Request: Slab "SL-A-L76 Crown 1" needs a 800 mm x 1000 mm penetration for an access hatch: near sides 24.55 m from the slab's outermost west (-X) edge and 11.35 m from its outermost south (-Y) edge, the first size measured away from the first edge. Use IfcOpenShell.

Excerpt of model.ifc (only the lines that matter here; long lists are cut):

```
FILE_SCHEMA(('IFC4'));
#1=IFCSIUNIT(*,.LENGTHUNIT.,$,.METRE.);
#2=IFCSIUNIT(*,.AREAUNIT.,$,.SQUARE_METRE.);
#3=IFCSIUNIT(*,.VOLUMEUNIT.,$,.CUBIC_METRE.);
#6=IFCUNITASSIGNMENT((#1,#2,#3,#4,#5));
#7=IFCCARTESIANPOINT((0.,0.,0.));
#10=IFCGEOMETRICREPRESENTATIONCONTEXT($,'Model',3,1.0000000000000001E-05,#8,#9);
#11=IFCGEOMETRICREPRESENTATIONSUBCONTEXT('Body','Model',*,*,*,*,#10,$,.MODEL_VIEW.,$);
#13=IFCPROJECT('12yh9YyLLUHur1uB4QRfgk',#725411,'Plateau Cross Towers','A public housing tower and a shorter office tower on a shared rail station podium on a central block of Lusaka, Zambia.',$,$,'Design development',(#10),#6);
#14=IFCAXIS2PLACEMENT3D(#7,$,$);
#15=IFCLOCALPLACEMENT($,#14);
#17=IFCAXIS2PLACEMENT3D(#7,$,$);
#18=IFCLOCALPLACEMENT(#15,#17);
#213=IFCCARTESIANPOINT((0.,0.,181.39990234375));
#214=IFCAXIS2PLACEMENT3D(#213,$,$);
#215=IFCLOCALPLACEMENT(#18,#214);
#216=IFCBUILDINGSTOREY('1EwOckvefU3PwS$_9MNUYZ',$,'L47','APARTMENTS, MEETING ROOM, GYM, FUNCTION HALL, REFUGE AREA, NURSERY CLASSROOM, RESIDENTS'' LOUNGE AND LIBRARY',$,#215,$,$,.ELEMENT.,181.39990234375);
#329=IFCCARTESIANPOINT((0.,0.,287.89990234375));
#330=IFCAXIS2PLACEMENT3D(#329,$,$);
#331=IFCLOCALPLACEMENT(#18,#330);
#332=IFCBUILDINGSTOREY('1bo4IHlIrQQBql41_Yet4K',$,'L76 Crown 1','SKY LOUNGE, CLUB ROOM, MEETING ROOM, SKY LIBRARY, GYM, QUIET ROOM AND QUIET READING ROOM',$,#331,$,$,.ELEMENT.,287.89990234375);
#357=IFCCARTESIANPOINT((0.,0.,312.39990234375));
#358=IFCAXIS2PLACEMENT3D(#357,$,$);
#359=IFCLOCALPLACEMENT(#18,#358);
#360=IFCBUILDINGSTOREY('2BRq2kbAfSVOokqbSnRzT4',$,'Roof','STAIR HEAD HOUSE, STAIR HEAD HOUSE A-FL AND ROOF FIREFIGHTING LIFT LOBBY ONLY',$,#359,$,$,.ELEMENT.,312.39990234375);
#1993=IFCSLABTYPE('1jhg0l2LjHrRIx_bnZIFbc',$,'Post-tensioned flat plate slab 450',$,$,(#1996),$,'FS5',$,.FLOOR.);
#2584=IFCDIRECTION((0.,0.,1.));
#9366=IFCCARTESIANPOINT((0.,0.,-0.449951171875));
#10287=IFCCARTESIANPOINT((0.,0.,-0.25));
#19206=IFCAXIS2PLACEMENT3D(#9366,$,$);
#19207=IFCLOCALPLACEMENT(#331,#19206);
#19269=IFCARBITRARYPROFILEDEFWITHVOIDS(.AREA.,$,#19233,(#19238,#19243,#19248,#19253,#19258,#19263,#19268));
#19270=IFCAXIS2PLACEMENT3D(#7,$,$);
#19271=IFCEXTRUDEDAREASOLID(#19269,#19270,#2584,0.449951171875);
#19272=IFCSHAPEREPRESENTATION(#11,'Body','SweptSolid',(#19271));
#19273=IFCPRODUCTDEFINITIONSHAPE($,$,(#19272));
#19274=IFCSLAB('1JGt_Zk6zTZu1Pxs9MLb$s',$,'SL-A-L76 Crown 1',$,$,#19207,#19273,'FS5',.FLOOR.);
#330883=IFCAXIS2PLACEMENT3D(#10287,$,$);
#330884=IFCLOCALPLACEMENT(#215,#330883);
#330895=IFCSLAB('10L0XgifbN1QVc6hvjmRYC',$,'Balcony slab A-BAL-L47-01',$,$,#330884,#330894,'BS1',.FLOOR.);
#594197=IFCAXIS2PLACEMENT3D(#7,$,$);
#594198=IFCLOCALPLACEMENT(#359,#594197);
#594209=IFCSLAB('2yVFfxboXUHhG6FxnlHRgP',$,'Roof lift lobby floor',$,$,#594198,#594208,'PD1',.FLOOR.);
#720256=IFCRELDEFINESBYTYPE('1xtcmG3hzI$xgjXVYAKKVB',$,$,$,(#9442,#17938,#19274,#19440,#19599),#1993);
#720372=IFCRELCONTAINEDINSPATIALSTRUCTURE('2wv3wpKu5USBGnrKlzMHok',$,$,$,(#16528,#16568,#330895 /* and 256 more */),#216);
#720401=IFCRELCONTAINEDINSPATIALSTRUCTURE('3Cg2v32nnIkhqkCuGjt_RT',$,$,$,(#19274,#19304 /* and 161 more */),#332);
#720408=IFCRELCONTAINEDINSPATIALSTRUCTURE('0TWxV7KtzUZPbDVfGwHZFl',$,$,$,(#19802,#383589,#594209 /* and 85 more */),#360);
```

```python
import numpy as np
import ifcopenshell
import ifcopenshell.api.feature
import ifcopenshell.api.geometry
import ifcopenshell.api.root
import ifcopenshell.geom
import ifcopenshell.util.placement
import ifcopenshell.util.representation
import ifcopenshell.util.shape
import ifcopenshell.util.unit

model = ifcopenshell.open("model.ifc")
unit_scale = ifcopenshell.util.unit.calculate_unit_scale(model)
settings = ifcopenshell.geom.settings()


def volume(element):
    """Net volume in cubic metres, openings subtracted."""
    shape = ifcopenshell.geom.create_shape(settings, element)
    return ifcopenshell.util.shape.get_volume(shape.geometry)


slab = model.by_guid("1JGt_Zk6zTZu1Pxs9MLb$s")
before = volume(slab)

# Extent in the slab's own axes, in metres. The edges named are its -X and -Y sides.
slab_shape = ifcopenshell.geom.create_shape(settings, slab)
vertices = ifcopenshell.util.shape.get_vertices(slab_shape.geometry)
x_min, y_min, bottom = vertices.min(axis=0)
top = vertices[:, 2].max()

opening = ifcopenshell.api.root.create_entity(model, ifc_class="IfcOpeningElement", name="Access hatch opening", predefined_type="OPENING")
context = ifcopenshell.util.representation.get_context(model, "Model", "Body", "MODEL_VIEW")
width, depth = 0.8, 1
outline = [(0.0, 0.0), (width, 0.0), (width, depth), (0.0, depth), (0.0, 0.0)]
# Overshoot both faces by 50 mm so the cut is clean.
shape = ifcopenshell.api.geometry.add_slab_representation(
    model, context=context, depth=top - bottom + 0.1, polyline=outline
)
ifcopenshell.api.geometry.assign_representation(model, product=opening, representation=shape)

matrix = ifcopenshell.util.placement.get_local_placement(slab.ObjectPlacement)
matrix[:, 3] = matrix @ np.append(np.array([x_min + 24.55, y_min + 11.35, bottom - 0.05]) / unit_scale, 1.0)
ifcopenshell.api.geometry.edit_object_placement(model, product=opening, matrix=matrix, is_si=False)
ifcopenshell.api.feature.add_feature(model, feature=opening, element=slab)

after = volume(slab)

print(f"slab volume {before:.3f} -> {after:.3f} m3")

model.write("model-out.ifc")
```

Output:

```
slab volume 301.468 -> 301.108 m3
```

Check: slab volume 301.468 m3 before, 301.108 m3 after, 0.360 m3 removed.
